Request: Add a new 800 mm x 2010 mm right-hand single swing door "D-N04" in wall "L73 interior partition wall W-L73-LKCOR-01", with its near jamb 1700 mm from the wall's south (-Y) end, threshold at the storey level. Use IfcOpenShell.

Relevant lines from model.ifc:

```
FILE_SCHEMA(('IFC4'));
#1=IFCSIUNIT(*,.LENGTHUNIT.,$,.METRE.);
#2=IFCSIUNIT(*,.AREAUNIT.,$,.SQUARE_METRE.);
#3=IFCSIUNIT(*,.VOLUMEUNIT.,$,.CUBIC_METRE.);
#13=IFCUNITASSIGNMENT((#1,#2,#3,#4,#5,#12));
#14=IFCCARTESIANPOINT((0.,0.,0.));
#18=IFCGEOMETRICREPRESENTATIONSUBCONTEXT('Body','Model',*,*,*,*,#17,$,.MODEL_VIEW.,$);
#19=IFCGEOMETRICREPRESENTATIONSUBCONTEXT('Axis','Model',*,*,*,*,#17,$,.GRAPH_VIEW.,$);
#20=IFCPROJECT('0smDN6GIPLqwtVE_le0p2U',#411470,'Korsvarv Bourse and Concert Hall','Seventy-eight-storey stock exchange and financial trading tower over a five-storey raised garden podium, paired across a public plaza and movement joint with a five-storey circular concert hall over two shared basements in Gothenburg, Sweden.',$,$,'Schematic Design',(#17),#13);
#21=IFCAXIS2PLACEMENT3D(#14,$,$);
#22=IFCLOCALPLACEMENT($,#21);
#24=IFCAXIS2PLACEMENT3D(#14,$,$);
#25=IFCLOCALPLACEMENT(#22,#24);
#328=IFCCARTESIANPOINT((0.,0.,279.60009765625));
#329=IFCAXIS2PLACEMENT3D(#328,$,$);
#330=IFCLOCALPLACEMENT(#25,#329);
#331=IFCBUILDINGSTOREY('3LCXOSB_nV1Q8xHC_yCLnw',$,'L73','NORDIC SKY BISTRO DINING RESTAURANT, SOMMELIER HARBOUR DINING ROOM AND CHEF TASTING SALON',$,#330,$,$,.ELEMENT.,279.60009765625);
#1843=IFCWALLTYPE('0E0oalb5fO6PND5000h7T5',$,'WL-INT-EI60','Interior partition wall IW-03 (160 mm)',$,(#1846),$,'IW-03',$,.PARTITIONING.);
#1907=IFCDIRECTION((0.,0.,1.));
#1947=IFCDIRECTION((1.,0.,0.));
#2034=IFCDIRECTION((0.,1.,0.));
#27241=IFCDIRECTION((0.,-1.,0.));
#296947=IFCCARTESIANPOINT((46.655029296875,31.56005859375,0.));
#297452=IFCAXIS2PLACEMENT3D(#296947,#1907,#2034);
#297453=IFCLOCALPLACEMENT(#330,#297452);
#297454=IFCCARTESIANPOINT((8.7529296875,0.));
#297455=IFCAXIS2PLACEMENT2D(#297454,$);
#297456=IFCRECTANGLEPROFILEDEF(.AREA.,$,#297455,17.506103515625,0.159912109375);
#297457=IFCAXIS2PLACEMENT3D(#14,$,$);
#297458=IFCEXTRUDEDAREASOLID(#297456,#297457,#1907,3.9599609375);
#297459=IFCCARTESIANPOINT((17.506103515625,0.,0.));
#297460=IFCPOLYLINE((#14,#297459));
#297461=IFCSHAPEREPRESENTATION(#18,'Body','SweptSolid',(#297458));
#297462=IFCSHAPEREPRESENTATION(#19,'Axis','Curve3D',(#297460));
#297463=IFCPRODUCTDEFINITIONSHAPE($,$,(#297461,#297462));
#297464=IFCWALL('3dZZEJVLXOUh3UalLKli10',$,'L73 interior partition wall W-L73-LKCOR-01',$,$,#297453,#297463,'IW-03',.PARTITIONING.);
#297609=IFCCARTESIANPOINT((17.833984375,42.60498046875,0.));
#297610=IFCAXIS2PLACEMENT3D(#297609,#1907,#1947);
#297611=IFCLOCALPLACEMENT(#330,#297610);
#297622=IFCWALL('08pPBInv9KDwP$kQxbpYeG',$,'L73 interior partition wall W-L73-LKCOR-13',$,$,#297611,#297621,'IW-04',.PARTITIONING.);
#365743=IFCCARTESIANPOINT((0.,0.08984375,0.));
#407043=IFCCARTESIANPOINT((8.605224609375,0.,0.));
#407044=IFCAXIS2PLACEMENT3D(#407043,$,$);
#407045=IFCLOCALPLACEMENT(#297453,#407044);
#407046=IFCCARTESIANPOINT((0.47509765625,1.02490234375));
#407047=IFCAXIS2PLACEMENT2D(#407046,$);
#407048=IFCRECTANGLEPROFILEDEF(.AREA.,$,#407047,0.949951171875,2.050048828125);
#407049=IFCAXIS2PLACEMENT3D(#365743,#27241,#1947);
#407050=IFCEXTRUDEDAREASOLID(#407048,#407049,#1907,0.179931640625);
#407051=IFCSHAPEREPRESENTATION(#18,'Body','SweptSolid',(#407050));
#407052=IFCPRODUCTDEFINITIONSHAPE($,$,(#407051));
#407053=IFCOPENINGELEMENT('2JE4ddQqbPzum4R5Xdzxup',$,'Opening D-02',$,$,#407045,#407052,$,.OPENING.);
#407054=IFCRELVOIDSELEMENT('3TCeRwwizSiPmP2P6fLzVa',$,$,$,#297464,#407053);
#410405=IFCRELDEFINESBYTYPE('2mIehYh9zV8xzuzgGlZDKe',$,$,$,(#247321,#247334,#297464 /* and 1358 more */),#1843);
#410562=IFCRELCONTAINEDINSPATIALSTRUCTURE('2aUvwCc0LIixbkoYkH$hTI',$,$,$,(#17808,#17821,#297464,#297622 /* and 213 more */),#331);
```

```python
import numpy as np
import ifcopenshell
import ifcopenshell.api.feature
import ifcopenshell.api.geometry
import ifcopenshell.api.root
import ifcopenshell.api.spatial
import ifcopenshell.geom
import ifcopenshell.util.element
import ifcopenshell.util.placement
import ifcopenshell.util.representation
import ifcopenshell.util.shape
import ifcopenshell.util.unit

model = ifcopenshell.open("model.ifc")
unit_scale = ifcopenshell.util.unit.calculate_unit_scale(model)
settings = ifcopenshell.geom.settings()


def volume(element):
    """Net volume in cubic metres, openings subtracted."""
    shape = ifcopenshell.geom.create_shape(settings, element)
    return ifcopenshell.util.shape.get_volume(shape.geometry)


wall = model.by_guid("3dZZEJVLXOUh3UalLKli10")
storey = ifcopenshell.util.element.get_container(wall, ifc_class="IfcBuildingStorey")
context = ifcopenshell.util.representation.get_context(model, "Model", "Body", "MODEL_VIEW")
before = volume(wall)

width, height, from_end, sill = 0.8, 2.01, 1.7, 0.0  # metres

# The wall runs along its own X axis, and the end named is its -X end.
wall_shape = ifcopenshell.geom.create_shape(settings, wall)
x, y, z = ifcopenshell.util.shape.get_vertices(wall_shape.geometry).T
start = x.min() + from_end
face, thickness = float(y.min()), float(y.max() - y.min())
wall_matrix = ifcopenshell.util.placement.get_local_placement(wall.ObjectPlacement)
level = ifcopenshell.util.placement.get_local_placement(storey.ObjectPlacement)[2, 3]


def in_wall(x, y):
    """Placement at x, y metres in the wall's axes, at sill height."""
    matrix = wall_matrix.copy()
    matrix[:, 3] = wall_matrix @ np.array([x / unit_scale, y / unit_scale, 0.0, 1.0])
    matrix[2, 3] = level + sill / unit_scale
    return matrix


# Opening: a box that overshoots both wall faces by 50 mm.
opening = ifcopenshell.api.root.create_entity(model, ifc_class="IfcOpeningElement", predefined_type="OPENING")
box = ifcopenshell.api.geometry.add_wall_representation(
    model, context=context, length=width, height=height, thickness=thickness + 0.1
)
ifcopenshell.api.geometry.assign_representation(model, product=opening, representation=box)
ifcopenshell.api.geometry.edit_object_placement(model, product=opening, matrix=in_wall(start, face - 0.05), is_si=False)
ifcopenshell.api.feature.add_feature(model, feature=opening, element=wall)

door = ifcopenshell.api.root.create_entity(model, ifc_class="IfcDoor", name="D-N04", predefined_type="DOOR")
door.OverallWidth, door.OverallHeight = width / unit_scale, height / unit_scale
door.OperationType = "SINGLE_SWING_RIGHT"
body = ifcopenshell.api.geometry.add_door_representation(
    model,
    context=context,
    overall_width=door.OverallWidth,
    overall_height=door.OverallHeight,
    operation_type="SINGLE_SWING_RIGHT",
    lining_properties={"LiningDepth": thickness / unit_scale, "ThresholdDepth": thickness / unit_scale},
)
ifcopenshell.api.geometry.assign_representation(model, product=door, representation=body)
ifcopenshell.api.spatial.assign_container(model, products=[door], relating_structure=storey)
ifcopenshell.api.feature.add_filling(model, opening=opening, element=door)

# The lining spans the wall, so the door starts at the wall face.
ifcopenshell.api.geometry.edit_object_placement(model, product=door, matrix=in_wall(start, face), is_si=False)

after = volume(wall)

print(f"wall volume {before:.3f} -> {after:.3f} m3")

model.write("model_updated.ifc")
```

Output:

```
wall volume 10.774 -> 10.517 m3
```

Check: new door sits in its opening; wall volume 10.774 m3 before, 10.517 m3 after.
